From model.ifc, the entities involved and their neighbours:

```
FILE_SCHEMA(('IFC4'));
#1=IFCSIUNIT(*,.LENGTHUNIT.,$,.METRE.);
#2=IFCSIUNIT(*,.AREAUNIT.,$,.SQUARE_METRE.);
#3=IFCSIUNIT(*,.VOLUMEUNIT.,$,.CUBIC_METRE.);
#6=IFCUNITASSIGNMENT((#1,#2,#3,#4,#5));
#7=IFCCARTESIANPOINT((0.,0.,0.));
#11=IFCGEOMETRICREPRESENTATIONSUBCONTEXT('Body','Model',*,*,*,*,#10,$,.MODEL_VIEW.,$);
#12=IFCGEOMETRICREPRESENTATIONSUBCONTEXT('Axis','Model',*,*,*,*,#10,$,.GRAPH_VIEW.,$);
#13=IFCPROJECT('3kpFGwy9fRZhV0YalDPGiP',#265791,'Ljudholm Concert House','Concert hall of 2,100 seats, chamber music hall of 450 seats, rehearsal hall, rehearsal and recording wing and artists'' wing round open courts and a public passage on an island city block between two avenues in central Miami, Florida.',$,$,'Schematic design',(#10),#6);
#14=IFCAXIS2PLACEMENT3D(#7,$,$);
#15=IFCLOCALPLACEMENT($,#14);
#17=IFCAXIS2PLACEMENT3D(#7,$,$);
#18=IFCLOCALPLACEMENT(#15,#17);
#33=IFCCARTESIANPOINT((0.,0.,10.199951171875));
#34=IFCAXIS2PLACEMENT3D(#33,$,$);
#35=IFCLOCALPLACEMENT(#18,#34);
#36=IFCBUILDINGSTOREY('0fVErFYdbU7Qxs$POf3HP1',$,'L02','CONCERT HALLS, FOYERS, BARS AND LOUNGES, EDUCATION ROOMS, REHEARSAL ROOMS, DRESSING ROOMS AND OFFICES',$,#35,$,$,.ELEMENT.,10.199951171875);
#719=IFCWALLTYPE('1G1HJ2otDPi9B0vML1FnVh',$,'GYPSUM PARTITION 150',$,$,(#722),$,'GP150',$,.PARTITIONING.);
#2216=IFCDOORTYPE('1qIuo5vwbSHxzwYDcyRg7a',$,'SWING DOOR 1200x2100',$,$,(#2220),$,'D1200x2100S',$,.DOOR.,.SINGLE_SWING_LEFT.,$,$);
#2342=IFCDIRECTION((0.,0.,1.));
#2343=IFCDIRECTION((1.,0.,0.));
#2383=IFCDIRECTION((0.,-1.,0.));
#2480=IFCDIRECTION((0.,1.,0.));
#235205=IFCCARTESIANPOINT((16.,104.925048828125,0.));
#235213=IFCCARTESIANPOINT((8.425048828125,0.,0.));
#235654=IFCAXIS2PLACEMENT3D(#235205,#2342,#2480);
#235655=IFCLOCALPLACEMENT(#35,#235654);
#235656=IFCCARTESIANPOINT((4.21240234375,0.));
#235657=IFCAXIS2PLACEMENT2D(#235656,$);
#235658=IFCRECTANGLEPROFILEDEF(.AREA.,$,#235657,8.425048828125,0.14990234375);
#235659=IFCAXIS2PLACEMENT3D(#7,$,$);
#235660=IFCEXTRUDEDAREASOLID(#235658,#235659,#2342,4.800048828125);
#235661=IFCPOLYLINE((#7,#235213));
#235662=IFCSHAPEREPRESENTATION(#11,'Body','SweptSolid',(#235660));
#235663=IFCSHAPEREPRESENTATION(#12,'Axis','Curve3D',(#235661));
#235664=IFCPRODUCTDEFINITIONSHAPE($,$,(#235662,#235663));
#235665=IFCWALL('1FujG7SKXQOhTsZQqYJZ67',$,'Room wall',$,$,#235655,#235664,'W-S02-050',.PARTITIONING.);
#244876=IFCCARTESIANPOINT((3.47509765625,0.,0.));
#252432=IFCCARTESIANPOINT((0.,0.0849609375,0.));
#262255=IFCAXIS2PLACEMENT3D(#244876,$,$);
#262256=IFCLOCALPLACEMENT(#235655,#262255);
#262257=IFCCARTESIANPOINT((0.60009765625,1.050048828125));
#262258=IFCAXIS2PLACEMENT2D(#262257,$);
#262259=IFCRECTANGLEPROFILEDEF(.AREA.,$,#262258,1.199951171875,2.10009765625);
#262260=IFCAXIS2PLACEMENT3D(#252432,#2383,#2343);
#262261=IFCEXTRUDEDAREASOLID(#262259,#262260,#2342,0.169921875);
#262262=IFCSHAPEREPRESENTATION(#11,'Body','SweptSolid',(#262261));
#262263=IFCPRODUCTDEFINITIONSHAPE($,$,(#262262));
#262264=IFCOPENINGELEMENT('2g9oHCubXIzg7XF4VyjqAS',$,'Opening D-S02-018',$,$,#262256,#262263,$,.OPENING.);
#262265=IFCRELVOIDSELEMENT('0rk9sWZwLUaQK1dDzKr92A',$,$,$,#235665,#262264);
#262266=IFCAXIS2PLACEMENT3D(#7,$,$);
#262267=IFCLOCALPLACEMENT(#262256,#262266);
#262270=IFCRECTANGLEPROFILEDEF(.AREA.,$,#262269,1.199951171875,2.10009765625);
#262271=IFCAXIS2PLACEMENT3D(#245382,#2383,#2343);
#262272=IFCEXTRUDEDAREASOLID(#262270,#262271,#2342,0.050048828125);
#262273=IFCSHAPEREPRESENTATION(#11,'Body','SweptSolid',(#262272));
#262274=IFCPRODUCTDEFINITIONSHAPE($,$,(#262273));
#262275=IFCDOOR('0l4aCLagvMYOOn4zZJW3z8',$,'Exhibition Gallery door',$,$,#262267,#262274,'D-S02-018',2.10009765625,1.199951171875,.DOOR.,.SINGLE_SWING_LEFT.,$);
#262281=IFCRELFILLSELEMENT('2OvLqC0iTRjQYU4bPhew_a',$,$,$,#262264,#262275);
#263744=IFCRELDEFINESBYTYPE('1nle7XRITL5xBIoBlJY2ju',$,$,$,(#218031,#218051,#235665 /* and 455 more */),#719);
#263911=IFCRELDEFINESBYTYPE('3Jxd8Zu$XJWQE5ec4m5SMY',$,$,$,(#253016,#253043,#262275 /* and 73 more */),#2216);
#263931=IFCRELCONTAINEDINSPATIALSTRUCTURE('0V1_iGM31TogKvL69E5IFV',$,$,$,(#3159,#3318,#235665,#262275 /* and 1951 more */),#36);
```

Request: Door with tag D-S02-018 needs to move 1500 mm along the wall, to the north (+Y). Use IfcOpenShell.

```python
import ifcopenshell
import ifcopenshell.api.geometry
import ifcopenshell.util.placement
import ifcopenshell.util.unit

model = ifcopenshell.open("model.ifc")
unit_scale = ifcopenshell.util.unit.calculate_unit_scale(model)

door = model.by_id(262275)
opening = door.FillsVoids[0].RelatingOpeningElement
wall = opening.VoidsElements[0].RelatingBuildingElement

wall_matrix = ifcopenshell.util.placement.get_local_placement(wall.ObjectPlacement)
shift = wall_matrix[:3, 0] * 1.5 / unit_scale
before = ifcopenshell.util.placement.get_local_placement(door.ObjectPlacement)[:3, 3].copy()

# The door is placed relative to its opening, so it follows when the opening moves.
matrix = ifcopenshell.util.placement.get_local_placement(opening.ObjectPlacement)
matrix[:3, 3] += shift
ifcopenshell.api.geometry.edit_object_placement(
    model, product=opening, matrix=matrix, is_si=False, should_transform_children=True
)

after = ifcopenshell.util.placement.get_local_placement(door.ObjectPlacement)[:3, 3]
print("door moved by", (after - before).round(3) + 0.0)

model.write("model_updated.ifc")
```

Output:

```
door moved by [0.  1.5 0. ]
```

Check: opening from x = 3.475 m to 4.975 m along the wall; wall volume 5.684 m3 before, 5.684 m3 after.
